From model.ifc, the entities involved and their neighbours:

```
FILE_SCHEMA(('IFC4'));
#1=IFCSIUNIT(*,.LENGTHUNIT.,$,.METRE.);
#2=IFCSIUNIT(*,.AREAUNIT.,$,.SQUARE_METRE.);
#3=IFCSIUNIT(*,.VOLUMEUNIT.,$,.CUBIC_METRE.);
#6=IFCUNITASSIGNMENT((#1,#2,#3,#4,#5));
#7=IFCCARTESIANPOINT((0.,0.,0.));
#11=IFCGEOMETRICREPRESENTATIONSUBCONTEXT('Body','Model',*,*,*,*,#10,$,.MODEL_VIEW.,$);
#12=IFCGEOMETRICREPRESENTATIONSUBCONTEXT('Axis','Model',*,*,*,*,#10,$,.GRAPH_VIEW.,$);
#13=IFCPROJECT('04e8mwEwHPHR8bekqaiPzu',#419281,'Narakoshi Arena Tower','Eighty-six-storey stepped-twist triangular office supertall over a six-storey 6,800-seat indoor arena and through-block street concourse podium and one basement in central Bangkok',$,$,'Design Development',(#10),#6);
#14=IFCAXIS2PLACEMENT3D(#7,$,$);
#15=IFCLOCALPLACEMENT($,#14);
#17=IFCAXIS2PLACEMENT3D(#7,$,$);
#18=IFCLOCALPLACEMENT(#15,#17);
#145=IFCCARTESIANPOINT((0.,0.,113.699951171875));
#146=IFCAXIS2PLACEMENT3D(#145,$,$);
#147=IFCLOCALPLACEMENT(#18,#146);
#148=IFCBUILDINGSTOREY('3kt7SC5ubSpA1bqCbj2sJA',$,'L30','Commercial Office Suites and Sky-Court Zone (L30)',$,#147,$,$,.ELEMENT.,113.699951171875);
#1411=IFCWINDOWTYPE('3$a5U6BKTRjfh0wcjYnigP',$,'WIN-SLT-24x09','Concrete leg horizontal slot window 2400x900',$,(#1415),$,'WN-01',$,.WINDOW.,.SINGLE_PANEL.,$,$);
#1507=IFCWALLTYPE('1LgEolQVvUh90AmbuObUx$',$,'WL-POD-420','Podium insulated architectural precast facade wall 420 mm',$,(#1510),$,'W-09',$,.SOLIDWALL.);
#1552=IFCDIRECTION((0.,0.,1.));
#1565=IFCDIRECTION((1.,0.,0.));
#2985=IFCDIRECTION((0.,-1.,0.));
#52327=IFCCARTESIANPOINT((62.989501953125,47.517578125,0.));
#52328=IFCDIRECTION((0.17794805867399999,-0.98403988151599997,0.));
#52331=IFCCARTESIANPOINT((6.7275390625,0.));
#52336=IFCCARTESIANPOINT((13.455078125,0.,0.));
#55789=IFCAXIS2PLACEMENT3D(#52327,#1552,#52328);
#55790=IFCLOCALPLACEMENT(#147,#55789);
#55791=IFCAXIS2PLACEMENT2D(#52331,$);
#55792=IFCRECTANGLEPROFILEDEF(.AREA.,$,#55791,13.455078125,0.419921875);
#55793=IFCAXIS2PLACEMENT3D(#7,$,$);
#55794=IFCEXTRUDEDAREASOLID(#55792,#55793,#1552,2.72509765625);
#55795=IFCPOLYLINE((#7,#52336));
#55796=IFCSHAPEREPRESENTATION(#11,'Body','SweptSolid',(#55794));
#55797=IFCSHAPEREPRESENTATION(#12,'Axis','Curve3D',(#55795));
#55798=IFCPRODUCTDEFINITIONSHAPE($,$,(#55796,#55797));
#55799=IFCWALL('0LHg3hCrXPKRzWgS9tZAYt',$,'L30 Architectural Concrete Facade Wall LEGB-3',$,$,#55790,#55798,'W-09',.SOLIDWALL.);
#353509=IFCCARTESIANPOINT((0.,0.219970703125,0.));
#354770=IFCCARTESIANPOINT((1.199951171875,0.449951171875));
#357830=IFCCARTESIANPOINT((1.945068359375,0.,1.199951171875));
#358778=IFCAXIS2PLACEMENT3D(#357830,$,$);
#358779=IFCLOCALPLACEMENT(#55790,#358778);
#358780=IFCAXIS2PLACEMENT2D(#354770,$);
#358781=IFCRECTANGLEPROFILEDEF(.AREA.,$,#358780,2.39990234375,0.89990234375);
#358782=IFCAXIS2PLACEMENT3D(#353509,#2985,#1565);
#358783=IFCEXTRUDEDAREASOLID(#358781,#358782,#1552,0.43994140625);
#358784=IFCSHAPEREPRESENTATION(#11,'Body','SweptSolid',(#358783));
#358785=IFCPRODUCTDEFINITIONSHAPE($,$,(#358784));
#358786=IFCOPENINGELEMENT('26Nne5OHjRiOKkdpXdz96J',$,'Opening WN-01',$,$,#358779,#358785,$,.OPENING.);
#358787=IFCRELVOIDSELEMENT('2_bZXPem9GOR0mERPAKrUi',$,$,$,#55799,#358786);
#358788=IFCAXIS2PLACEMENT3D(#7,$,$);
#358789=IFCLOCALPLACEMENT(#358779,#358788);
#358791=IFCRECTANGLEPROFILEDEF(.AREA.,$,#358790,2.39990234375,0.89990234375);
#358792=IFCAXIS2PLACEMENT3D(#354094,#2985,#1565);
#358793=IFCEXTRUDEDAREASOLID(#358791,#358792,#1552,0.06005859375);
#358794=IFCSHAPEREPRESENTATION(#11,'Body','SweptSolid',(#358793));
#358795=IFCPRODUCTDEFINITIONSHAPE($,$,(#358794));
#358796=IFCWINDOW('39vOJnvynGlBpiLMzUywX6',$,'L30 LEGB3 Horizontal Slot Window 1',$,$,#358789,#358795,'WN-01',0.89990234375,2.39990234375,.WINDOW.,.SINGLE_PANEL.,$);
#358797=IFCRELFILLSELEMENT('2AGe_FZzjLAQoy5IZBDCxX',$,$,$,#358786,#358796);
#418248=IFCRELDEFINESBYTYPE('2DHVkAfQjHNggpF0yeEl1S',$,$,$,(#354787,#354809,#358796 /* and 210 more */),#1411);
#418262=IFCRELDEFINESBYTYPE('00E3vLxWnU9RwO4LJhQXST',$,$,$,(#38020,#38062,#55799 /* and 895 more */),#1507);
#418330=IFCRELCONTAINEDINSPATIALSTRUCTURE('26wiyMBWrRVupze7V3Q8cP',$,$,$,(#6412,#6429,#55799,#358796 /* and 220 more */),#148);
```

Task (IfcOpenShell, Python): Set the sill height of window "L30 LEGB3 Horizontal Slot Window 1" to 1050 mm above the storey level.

```python
import numpy as np
import ifcopenshell
import ifcopenshell.api.geometry
import ifcopenshell.geom
import ifcopenshell.util.element
import ifcopenshell.util.placement
import ifcopenshell.util.shape
import ifcopenshell.util.unit

model = ifcopenshell.open("model.ifc")
unit_scale = ifcopenshell.util.unit.calculate_unit_scale(model)

window = model.by_id(358796)
opening = window.FillsVoids[0].RelatingOpeningElement
storey = ifcopenshell.util.element.get_container(window, ifc_class="IfcBuildingStorey")
level = ifcopenshell.util.placement.get_local_placement(storey.ObjectPlacement)[2, 3]

# The opening's origin need not be at the sill, so measure its lowest point.
shape = ifcopenshell.geom.create_shape(ifcopenshell.geom.settings(), opening)
bottom = ifcopenshell.util.shape.get_shape_bottom_elevation(shape, shape.geometry) / unit_scale
dz = level + 1.05 / unit_scale - bottom

shift = np.array([0.0, 0.0, dz])
# The window is placed relative to its opening, so it follows when the opening moves.
matrix = ifcopenshell.util.placement.get_local_placement(opening.ObjectPlacement)
matrix[:3, 3] += shift
ifcopenshell.api.geometry.edit_object_placement(
    model, product=opening, matrix=matrix, is_si=False, should_transform_children=True
)

print(f"moved by {dz * unit_scale:+.3f} m")

model.write("model_rev.ifc")
```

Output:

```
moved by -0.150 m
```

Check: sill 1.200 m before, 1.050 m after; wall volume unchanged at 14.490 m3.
